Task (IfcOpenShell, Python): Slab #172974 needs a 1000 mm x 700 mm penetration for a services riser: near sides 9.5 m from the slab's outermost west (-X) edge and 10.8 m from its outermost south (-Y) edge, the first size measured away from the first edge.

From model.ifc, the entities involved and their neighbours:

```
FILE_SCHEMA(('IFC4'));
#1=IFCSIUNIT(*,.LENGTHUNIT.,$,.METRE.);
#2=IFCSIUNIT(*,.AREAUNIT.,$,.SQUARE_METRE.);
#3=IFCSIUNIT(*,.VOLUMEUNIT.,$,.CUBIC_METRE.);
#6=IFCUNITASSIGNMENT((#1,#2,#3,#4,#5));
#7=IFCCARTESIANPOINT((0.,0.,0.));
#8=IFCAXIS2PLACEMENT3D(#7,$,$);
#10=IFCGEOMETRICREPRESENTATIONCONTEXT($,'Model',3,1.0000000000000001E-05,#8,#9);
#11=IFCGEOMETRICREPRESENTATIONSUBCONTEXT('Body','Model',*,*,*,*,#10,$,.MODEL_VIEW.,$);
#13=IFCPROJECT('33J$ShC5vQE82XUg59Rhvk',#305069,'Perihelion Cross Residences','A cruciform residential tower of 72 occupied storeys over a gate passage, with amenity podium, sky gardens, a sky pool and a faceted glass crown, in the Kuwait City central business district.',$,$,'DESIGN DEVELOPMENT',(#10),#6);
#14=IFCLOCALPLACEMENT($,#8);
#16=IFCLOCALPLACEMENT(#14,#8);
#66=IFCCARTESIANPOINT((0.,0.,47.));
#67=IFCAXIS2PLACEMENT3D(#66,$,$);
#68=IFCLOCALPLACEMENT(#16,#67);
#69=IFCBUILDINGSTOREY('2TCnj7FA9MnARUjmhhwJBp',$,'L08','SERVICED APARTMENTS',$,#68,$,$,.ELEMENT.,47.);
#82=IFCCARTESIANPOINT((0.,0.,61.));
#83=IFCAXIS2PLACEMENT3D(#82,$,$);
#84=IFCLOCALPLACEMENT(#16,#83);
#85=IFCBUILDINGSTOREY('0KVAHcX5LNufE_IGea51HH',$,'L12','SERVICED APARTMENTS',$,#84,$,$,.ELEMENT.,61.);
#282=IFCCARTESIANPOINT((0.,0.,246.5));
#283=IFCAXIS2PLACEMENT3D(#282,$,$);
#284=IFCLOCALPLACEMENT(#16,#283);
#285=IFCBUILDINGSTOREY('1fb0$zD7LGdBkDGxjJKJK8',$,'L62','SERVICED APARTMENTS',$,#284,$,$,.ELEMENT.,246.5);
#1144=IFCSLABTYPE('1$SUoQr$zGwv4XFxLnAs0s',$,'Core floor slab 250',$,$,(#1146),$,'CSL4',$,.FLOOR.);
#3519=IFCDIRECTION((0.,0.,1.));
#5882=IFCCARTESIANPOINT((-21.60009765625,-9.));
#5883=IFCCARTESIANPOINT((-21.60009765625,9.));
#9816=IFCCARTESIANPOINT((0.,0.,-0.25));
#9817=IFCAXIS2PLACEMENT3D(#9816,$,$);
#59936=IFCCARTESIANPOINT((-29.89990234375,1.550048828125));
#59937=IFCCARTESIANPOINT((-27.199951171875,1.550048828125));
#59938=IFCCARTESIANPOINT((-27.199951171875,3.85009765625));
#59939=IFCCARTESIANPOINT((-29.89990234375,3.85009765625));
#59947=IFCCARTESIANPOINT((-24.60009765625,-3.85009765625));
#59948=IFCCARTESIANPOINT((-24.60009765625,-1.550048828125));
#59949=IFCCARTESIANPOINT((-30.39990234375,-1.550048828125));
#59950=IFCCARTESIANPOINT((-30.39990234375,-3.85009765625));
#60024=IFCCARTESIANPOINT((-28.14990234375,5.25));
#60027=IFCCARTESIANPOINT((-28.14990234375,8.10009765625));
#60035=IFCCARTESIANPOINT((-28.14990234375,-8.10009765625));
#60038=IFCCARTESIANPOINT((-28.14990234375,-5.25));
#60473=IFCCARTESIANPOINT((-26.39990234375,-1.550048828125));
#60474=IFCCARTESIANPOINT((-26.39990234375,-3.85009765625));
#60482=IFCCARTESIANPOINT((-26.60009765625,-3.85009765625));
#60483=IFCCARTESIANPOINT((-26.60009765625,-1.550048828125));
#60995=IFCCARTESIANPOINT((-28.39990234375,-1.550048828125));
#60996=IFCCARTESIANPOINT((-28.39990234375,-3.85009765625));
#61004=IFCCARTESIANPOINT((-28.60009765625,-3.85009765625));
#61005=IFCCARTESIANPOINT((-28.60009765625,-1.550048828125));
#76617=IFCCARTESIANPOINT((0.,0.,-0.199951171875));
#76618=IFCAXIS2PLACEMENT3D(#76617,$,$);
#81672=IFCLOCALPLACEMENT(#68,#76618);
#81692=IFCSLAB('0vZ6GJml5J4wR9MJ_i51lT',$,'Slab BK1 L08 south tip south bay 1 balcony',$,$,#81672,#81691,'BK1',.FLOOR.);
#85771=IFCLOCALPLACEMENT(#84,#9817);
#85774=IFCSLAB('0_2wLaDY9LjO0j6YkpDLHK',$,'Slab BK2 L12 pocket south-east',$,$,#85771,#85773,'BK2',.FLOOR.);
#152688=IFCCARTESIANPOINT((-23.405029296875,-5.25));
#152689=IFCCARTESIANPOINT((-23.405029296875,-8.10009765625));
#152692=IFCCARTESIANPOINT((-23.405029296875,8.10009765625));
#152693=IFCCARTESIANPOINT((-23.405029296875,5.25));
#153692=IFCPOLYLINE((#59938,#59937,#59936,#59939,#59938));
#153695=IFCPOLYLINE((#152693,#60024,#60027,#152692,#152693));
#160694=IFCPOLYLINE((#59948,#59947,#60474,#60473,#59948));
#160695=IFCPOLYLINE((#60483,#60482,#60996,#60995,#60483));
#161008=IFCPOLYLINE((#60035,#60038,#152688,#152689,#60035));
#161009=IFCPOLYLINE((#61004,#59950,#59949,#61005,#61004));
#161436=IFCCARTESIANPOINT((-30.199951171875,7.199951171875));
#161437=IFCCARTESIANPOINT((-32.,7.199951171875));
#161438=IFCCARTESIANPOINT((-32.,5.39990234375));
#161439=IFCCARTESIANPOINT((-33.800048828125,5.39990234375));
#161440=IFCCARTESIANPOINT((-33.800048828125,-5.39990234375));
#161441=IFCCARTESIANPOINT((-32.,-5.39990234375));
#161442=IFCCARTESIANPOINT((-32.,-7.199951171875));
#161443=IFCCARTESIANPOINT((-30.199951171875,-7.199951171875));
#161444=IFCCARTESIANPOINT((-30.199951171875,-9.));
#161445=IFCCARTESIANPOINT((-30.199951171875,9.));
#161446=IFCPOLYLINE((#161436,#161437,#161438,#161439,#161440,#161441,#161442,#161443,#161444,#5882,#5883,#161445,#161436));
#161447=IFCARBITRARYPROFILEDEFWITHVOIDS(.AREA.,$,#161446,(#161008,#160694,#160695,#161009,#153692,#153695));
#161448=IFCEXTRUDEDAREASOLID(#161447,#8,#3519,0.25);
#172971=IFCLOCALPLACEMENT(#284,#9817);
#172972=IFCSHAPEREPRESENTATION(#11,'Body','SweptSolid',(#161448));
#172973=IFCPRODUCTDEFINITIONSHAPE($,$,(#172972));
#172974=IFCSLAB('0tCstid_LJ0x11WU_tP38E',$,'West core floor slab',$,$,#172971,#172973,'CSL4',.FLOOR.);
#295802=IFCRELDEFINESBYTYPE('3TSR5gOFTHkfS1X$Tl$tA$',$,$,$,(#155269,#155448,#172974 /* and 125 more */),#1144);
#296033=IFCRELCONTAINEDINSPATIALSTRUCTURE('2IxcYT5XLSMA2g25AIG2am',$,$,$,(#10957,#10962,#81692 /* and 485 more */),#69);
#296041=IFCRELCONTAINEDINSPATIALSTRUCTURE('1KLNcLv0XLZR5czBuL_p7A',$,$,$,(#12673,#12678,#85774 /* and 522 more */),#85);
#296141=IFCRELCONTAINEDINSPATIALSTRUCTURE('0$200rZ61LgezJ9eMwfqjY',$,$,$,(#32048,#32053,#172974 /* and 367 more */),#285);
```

```python
import numpy as np
import ifcopenshell
import ifcopenshell.api.feature
import ifcopenshell.api.geometry
import ifcopenshell.api.root
import ifcopenshell.geom
import ifcopenshell.util.placement
import ifcopenshell.util.representation
import ifcopenshell.util.shape
import ifcopenshell.util.unit

model = ifcopenshell.open("model.ifc")
unit_scale = ifcopenshell.util.unit.calculate_unit_scale(model)
settings = ifcopenshell.geom.settings()


def volume(element):
    """Net volume in cubic metres, openings subtracted."""
    shape = ifcopenshell.geom.create_shape(settings, element)
    return ifcopenshell.util.shape.get_volume(shape.geometry)


slab = model.by_guid("0tCstid_LJ0x11WU_tP38E")
before = volume(slab)

# Extent in the slab's own axes, in metres. The edges named are its -X and -Y sides.
slab_shape = ifcopenshell.geom.create_shape(settings, slab)
vertices = ifcopenshell.util.shape.get_vertices(slab_shape.geometry)
x_min, y_min, bottom = vertices.min(axis=0)
top = vertices[:, 2].max()

opening = ifcopenshell.api.root.create_entity(model, ifc_class="IfcOpeningElement", name="Services riser opening", predefined_type="OPENING")
context = ifcopenshell.util.representation.get_context(model, "Model", "Body", "MODEL_VIEW")
width, depth = 1, 0.7
outline = [(0.0, 0.0), (width, 0.0), (width, depth), (0.0, depth), (0.0, 0.0)]
# Overshoot both faces by 50 mm so the cut is clean.
shape = ifcopenshell.api.geometry.add_slab_representation(
    model, context=context, depth=top - bottom + 0.1, polyline=outline
)
ifcopenshell.api.geometry.assign_representation(model, product=opening, representation=shape)

matrix = ifcopenshell.util.placement.get_local_placement(slab.ObjectPlacement)
matrix[:, 3] = matrix @ np.append(np.array([x_min + 9.5, y_min + 10.8, bottom - 0.05]) / unit_scale, 1.0)
ifcopenshell.api.geometry.edit_object_placement(model, product=opening, matrix=matrix, is_si=False)
ifcopenshell.api.feature.add_feature(model, feature=opening, element=slab)

after = volume(slab)

print(f"slab volume {before:.3f} -> {after:.3f} m3")

model.write("model_v2.ifc")
```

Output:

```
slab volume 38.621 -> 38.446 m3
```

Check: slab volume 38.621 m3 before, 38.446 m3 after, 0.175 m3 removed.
